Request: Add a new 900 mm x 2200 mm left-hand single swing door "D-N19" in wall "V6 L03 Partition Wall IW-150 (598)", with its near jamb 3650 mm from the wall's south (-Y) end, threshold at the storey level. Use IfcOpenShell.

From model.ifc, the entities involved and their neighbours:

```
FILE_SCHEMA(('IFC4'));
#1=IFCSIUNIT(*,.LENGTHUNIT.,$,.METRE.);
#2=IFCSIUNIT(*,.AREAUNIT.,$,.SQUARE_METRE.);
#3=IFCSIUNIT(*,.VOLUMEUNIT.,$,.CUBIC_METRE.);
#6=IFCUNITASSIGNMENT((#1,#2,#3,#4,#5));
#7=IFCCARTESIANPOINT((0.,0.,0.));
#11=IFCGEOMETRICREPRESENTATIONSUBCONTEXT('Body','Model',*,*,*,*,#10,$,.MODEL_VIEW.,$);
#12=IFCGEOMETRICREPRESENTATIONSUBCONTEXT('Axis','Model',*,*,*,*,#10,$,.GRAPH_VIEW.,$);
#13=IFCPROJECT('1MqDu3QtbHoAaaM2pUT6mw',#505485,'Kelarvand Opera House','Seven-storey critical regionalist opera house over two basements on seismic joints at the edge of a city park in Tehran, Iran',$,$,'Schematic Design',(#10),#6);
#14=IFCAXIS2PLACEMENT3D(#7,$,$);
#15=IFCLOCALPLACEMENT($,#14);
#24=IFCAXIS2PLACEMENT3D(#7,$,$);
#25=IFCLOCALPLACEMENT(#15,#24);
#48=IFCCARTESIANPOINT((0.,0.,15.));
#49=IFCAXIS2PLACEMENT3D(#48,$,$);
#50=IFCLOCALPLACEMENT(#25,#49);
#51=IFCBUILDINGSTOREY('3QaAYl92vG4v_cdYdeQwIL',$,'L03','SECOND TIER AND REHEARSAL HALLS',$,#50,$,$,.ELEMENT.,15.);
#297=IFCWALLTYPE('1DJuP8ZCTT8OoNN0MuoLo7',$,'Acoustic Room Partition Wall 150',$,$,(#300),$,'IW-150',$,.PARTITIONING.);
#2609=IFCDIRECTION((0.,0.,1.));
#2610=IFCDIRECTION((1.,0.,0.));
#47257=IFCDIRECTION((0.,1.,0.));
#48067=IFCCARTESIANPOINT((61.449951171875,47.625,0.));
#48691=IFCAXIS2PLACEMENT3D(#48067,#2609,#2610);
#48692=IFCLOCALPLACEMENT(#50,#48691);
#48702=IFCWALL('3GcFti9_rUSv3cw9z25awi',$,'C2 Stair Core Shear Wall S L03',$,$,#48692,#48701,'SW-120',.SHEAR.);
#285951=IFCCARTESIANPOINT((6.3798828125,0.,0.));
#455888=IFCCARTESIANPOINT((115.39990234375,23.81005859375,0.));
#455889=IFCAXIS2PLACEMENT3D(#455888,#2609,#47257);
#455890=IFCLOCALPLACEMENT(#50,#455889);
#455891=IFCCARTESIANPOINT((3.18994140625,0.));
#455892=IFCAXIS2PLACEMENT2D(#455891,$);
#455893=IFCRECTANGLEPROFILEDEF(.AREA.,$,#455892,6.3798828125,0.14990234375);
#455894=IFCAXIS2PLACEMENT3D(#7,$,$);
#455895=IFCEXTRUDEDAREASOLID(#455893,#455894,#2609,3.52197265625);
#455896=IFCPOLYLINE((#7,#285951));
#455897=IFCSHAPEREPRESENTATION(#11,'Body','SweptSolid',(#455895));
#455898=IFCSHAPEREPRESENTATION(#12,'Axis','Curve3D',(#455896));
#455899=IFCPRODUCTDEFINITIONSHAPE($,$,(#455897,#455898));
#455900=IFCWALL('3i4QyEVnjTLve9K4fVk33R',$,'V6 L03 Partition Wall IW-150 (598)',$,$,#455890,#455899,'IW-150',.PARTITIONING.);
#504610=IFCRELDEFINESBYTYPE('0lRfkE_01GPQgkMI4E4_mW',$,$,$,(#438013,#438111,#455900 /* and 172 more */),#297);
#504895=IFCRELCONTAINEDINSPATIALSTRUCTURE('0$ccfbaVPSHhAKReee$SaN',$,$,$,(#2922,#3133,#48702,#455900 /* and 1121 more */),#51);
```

```python
import numpy as np
import ifcopenshell
import ifcopenshell.api.feature
import ifcopenshell.api.geometry
import ifcopenshell.api.root
import ifcopenshell.api.spatial
import ifcopenshell.geom
import ifcopenshell.util.element
import ifcopenshell.util.placement
import ifcopenshell.util.representation
import ifcopenshell.util.shape
import ifcopenshell.util.unit

model = ifcopenshell.open("model.ifc")
unit_scale = ifcopenshell.util.unit.calculate_unit_scale(model)
settings = ifcopenshell.geom.settings()


def volume(element):
    """Net volume in cubic metres, openings subtracted."""
    shape = ifcopenshell.geom.create_shape(settings, element)
    return ifcopenshell.util.shape.get_volume(shape.geometry)


wall = model.by_guid("3i4QyEVnjTLve9K4fVk33R")
storey = ifcopenshell.util.element.get_container(wall, ifc_class="IfcBuildingStorey")
context = ifcopenshell.util.representation.get_context(model, "Model", "Body", "MODEL_VIEW")
before = volume(wall)

width, height, from_end, sill = 0.9, 2.2, 3.65, 0.0  # metres

# The wall runs along its own X axis, and the end named is its -X end.
wall_shape = ifcopenshell.geom.create_shape(settings, wall)
x, y, z = ifcopenshell.util.shape.get_vertices(wall_shape.geometry).T
start = x.min() + from_end
face, thickness = float(y.min()), float(y.max() - y.min())
wall_matrix = ifcopenshell.util.placement.get_local_placement(wall.ObjectPlacement)
level = ifcopenshell.util.placement.get_local_placement(storey.ObjectPlacement)[2, 3]


def in_wall(x, y):
    """Placement at x, y metres in the wall's axes, at sill height."""
    matrix = wall_matrix.copy()
    matrix[:, 3] = wall_matrix @ np.array([x / unit_scale, y / unit_scale, 0.0, 1.0])
    matrix[2, 3] = level + sill / unit_scale
    return matrix


# Opening: a box that overshoots both wall faces by 50 mm.
opening = ifcopenshell.api.root.create_entity(model, ifc_class="IfcOpeningElement", predefined_type="OPENING")
box = ifcopenshell.api.geometry.add_wall_representation(
    model, context=context, length=width, height=height, thickness=thickness + 0.1
)
ifcopenshell.api.geometry.assign_representation(model, product=opening, representation=box)
ifcopenshell.api.geometry.edit_object_placement(model, product=opening, matrix=in_wall(start, face - 0.05), is_si=False)
ifcopenshell.api.feature.add_feature(model, feature=opening, element=wall)

door = ifcopenshell.api.root.create_entity(model, ifc_class="IfcDoor", name="D-N19", predefined_type="DOOR")
door.OverallWidth, door.OverallHeight = width / unit_scale, height / unit_scale
door.OperationType = "SINGLE_SWING_LEFT"
body = ifcopenshell.api.geometry.add_door_representation(
    model,
    context=context,
    overall_width=door.OverallWidth,
    overall_height=door.OverallHeight,
    operation_type="SINGLE_SWING_LEFT",
    lining_properties={"LiningDepth": thickness / unit_scale, "ThresholdDepth": thickness / unit_scale},
)
ifcopenshell.api.geometry.assign_representation(model, product=door, representation=body)
ifcopenshell.api.spatial.assign_container(model, products=[door], relating_structure=storey)
ifcopenshell.api.feature.add_filling(model, opening=opening, element=door)

# The lining spans the wall, so the door starts at the wall face.
ifcopenshell.api.geometry.edit_object_placement(model, product=door, matrix=in_wall(start, face), is_si=False)

after = volume(wall)

print(f"wall volume {before:.3f} -> {after:.3f} m3")

model.write("model_v2.ifc")
```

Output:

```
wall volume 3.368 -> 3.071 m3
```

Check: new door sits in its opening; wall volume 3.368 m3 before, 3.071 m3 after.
